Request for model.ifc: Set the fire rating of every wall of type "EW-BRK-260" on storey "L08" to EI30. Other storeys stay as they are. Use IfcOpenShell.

First a look at what the model holds.

```python
import ifcopenshell
import ifcopenshell.util.element

model = ifcopenshell.open("model.ifc")
print(model.schema)
storey = next(s for s in model.by_type("IfcBuildingStorey") if s.Name == "L08")
walls = [e for e in ifcopenshell.util.element.get_decomposition(storey) if e.is_a("IfcWall")]
seen = {}
for e in walls:
    element_type = ifcopenshell.util.element.get_type(e)
    key = (element_type.Name if element_type != e and element_type else None, ifcopenshell.util.element.get_pset(e, "Pset_WallCommon", "FireRating"))
    seen[key] = seen.get(key, 0) + 1
for (name, value), count in sorted(seen.items(), key=str):
    print(count, "x", name, "|", value)
```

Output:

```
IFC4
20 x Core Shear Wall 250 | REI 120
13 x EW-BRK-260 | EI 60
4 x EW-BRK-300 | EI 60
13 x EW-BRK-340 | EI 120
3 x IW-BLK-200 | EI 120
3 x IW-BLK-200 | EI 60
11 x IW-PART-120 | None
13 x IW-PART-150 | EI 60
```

```python
import ifcopenshell
import ifcopenshell.api.pset
import ifcopenshell.util.element

model = ifcopenshell.open("model.ifc")

storey = next(s for s in model.by_type("IfcBuildingStorey") if s.Name == "L08")
walls = [e for e in ifcopenshell.util.element.get_decomposition(storey) if e.is_a("IfcWall")]

count = 0
for e in walls:
    element_type = ifcopenshell.util.element.get_type(e)
    if element_type in (None, e) or element_type.Name != "EW-BRK-260":
        continue
    # add_pset returns the element's existing set when there is one.
    pset = ifcopenshell.api.pset.add_pset(model, product=e, name="Pset_WallCommon")
    ifcopenshell.api.pset.edit_pset(model, pset=pset, properties={"FireRating": "EI30"})
    count += 1

print(count, "walls updated")

model.write("model_v2.ifc")
```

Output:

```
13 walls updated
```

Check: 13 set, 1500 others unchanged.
